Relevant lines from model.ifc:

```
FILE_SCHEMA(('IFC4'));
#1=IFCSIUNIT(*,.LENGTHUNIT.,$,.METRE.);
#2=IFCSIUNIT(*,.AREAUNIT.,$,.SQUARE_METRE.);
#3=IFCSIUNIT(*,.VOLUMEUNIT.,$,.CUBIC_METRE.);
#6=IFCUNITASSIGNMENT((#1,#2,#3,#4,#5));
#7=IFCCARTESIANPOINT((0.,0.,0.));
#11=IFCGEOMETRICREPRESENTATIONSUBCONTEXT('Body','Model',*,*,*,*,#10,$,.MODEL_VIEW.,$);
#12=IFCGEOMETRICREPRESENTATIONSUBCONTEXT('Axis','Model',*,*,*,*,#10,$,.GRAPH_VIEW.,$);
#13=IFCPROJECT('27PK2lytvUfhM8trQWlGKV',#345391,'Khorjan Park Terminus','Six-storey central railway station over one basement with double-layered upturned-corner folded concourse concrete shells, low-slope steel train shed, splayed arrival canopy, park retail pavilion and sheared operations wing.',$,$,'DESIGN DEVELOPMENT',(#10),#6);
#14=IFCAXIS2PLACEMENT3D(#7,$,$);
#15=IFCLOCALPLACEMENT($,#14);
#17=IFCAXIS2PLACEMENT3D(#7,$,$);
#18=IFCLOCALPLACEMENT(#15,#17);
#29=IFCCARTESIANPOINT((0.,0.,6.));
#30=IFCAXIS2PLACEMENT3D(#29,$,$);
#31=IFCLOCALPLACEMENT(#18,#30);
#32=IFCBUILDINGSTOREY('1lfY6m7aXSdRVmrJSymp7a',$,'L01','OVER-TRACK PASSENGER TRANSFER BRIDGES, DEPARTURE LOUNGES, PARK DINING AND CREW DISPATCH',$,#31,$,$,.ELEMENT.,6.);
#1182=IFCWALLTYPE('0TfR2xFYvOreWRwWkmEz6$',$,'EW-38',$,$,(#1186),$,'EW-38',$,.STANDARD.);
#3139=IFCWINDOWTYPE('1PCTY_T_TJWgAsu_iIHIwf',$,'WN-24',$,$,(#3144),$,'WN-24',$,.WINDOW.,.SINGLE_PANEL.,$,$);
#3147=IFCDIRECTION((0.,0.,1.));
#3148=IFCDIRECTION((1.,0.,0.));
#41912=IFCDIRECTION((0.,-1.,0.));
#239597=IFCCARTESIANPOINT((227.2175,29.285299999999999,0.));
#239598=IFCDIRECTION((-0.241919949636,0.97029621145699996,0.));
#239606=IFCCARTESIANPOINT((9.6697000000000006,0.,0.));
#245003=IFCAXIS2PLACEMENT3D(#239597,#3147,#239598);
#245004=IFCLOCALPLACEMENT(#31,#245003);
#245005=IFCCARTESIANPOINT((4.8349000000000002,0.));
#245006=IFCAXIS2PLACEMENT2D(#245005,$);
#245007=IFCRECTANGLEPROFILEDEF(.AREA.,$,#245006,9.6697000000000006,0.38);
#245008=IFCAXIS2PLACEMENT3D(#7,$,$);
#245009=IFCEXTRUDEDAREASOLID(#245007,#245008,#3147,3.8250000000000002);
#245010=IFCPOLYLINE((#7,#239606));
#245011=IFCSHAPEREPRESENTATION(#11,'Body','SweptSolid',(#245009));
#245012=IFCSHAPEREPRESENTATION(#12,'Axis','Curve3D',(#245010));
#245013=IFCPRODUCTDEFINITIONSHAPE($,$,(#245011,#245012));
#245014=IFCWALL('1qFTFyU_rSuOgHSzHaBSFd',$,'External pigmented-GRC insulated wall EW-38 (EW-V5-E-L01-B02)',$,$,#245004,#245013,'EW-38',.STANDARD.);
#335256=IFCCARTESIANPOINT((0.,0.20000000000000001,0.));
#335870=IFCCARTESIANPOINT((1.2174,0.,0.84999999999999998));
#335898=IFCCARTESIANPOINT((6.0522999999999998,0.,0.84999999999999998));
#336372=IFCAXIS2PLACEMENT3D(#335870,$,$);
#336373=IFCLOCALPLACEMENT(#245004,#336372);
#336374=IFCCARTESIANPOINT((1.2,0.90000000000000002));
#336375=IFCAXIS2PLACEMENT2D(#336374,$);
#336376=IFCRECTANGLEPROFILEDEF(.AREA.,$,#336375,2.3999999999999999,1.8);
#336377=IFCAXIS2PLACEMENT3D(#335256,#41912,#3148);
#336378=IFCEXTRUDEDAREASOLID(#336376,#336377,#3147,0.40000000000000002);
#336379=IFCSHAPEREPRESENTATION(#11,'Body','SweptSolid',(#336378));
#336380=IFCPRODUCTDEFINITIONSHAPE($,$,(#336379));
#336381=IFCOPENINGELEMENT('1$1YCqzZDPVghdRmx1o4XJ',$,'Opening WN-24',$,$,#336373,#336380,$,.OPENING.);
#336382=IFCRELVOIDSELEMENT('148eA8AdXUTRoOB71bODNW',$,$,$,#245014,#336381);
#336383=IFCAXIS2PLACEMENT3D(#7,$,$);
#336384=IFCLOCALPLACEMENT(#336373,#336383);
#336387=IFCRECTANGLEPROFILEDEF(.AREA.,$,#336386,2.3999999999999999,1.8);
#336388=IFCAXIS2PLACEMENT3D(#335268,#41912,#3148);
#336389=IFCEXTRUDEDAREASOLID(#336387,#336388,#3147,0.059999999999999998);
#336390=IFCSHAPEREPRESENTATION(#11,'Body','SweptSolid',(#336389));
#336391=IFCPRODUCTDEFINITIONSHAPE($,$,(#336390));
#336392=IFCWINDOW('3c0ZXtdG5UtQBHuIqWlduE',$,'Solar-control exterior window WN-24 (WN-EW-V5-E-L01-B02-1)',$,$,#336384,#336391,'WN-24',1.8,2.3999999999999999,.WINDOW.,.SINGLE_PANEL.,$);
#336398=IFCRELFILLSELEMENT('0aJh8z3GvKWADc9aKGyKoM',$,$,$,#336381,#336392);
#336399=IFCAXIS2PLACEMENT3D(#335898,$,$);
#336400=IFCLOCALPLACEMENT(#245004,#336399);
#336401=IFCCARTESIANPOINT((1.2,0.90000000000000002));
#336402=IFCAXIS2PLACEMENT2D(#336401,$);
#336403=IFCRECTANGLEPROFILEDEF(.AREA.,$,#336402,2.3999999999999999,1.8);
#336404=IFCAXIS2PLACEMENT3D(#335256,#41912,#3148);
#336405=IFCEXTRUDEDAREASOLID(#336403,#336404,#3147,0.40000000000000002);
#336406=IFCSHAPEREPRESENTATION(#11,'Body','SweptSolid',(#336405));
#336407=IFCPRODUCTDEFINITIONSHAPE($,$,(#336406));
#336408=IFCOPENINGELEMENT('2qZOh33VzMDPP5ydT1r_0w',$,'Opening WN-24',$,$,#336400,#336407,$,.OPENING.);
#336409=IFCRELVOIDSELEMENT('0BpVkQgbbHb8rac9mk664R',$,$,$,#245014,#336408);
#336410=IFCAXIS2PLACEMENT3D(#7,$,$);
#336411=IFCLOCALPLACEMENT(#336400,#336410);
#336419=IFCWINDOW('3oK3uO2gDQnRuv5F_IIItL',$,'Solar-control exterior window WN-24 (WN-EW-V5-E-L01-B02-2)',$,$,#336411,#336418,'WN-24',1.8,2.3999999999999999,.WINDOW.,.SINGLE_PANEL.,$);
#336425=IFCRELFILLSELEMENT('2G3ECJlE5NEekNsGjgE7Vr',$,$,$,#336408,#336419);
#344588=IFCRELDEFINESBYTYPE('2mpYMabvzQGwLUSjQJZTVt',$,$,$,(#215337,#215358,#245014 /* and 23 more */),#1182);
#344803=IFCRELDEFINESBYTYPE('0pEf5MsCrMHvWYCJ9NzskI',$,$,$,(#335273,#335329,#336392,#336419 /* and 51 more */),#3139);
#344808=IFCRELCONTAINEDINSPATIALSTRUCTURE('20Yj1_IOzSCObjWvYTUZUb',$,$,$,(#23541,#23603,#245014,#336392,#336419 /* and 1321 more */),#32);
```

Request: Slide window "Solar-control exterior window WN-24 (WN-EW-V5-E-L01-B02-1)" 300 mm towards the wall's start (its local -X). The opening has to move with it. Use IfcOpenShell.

```python
import ifcopenshell
import ifcopenshell.api.geometry
import ifcopenshell.util.placement

model = ifcopenshell.open("model.ifc")

window = model.by_guid("3c0ZXtdG5UtQBHuIqWlduE")
opening = window.FillsVoids[0].RelatingOpeningElement
wall = opening.VoidsElements[0].RelatingBuildingElement

wall_matrix = ifcopenshell.util.placement.get_local_placement(wall.ObjectPlacement)
shift = wall_matrix[:3, 0] * -0.3
before = ifcopenshell.util.placement.get_local_placement(window.ObjectPlacement)[:3, 3].copy()

# The window is placed relative to its opening, so it follows when the opening moves.
matrix = ifcopenshell.util.placement.get_local_placement(opening.ObjectPlacement)
matrix[:3, 3] += shift
ifcopenshell.api.geometry.edit_object_placement(
    model, product=opening, matrix=matrix, is_si=False, should_transform_children=True
)

after = ifcopenshell.util.placement.get_local_placement(window.ObjectPlacement)[:3, 3]
print("window moved by", (after - before).round(3) + 0.0)

model.write("model-out.ifc")
```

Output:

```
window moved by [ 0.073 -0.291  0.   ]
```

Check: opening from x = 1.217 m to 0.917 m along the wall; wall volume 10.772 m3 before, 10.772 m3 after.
